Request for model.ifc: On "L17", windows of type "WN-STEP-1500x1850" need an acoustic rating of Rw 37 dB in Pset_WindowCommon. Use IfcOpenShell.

First a look at what the model holds.

```python
import ifcopenshell
import ifcopenshell.util.element

model = ifcopenshell.open("model.ifc")
print(model.schema)
storey = next(s for s in model.by_type("IfcBuildingStorey") if s.Name == "L17")
windows = [e for e in ifcopenshell.util.element.get_decomposition(storey) if e.is_a("IfcWindow")]
seen = {}
for e in windows:
    element_type = ifcopenshell.util.element.get_type(e)
    key = (element_type.Name if element_type != e and element_type else None, ifcopenshell.util.element.get_pset(e, "Pset_WindowCommon", "AcousticRating"))
    seen[key] = seen.get(key, 0) + 1
for (name, value), count in sorted(seen.items(), key=str):
    print(count, "x", name, "|", value)
```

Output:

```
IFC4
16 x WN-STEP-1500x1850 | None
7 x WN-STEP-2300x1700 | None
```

```python
import ifcopenshell
import ifcopenshell.api.pset
import ifcopenshell.util.element

model = ifcopenshell.open("model.ifc")

storey = next(s for s in model.by_type("IfcBuildingStorey") if s.Name == "L17")
windows = [e for e in ifcopenshell.util.element.get_decomposition(storey) if e.is_a("IfcWindow")]

count = 0
for e in windows:
    element_type = ifcopenshell.util.element.get_type(e)
    if element_type in (None, e) or element_type.Name != "WN-STEP-1500x1850":
        continue
    found = ifcopenshell.util.element.get_pset(e, "Pset_WindowCommon", should_inherit=False)
    if found:
        pset = model.by_id(found["id"])
        if len(ifcopenshell.util.element.get_elements_by_pset(pset)) > 1:
            pset = ifcopenshell.api.pset.unshare_pset(model, products=[e], pset=pset)[0]
    else:
        pset = ifcopenshell.api.pset.add_pset(model, product=e, name="Pset_WindowCommon")
    ifcopenshell.api.pset.edit_pset(model, pset=pset, properties={"AcousticRating": "Rw 37 dB"})
    count += 1

print(count, "windows updated")

model.write("model_rev.ifc")
```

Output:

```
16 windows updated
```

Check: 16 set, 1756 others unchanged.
